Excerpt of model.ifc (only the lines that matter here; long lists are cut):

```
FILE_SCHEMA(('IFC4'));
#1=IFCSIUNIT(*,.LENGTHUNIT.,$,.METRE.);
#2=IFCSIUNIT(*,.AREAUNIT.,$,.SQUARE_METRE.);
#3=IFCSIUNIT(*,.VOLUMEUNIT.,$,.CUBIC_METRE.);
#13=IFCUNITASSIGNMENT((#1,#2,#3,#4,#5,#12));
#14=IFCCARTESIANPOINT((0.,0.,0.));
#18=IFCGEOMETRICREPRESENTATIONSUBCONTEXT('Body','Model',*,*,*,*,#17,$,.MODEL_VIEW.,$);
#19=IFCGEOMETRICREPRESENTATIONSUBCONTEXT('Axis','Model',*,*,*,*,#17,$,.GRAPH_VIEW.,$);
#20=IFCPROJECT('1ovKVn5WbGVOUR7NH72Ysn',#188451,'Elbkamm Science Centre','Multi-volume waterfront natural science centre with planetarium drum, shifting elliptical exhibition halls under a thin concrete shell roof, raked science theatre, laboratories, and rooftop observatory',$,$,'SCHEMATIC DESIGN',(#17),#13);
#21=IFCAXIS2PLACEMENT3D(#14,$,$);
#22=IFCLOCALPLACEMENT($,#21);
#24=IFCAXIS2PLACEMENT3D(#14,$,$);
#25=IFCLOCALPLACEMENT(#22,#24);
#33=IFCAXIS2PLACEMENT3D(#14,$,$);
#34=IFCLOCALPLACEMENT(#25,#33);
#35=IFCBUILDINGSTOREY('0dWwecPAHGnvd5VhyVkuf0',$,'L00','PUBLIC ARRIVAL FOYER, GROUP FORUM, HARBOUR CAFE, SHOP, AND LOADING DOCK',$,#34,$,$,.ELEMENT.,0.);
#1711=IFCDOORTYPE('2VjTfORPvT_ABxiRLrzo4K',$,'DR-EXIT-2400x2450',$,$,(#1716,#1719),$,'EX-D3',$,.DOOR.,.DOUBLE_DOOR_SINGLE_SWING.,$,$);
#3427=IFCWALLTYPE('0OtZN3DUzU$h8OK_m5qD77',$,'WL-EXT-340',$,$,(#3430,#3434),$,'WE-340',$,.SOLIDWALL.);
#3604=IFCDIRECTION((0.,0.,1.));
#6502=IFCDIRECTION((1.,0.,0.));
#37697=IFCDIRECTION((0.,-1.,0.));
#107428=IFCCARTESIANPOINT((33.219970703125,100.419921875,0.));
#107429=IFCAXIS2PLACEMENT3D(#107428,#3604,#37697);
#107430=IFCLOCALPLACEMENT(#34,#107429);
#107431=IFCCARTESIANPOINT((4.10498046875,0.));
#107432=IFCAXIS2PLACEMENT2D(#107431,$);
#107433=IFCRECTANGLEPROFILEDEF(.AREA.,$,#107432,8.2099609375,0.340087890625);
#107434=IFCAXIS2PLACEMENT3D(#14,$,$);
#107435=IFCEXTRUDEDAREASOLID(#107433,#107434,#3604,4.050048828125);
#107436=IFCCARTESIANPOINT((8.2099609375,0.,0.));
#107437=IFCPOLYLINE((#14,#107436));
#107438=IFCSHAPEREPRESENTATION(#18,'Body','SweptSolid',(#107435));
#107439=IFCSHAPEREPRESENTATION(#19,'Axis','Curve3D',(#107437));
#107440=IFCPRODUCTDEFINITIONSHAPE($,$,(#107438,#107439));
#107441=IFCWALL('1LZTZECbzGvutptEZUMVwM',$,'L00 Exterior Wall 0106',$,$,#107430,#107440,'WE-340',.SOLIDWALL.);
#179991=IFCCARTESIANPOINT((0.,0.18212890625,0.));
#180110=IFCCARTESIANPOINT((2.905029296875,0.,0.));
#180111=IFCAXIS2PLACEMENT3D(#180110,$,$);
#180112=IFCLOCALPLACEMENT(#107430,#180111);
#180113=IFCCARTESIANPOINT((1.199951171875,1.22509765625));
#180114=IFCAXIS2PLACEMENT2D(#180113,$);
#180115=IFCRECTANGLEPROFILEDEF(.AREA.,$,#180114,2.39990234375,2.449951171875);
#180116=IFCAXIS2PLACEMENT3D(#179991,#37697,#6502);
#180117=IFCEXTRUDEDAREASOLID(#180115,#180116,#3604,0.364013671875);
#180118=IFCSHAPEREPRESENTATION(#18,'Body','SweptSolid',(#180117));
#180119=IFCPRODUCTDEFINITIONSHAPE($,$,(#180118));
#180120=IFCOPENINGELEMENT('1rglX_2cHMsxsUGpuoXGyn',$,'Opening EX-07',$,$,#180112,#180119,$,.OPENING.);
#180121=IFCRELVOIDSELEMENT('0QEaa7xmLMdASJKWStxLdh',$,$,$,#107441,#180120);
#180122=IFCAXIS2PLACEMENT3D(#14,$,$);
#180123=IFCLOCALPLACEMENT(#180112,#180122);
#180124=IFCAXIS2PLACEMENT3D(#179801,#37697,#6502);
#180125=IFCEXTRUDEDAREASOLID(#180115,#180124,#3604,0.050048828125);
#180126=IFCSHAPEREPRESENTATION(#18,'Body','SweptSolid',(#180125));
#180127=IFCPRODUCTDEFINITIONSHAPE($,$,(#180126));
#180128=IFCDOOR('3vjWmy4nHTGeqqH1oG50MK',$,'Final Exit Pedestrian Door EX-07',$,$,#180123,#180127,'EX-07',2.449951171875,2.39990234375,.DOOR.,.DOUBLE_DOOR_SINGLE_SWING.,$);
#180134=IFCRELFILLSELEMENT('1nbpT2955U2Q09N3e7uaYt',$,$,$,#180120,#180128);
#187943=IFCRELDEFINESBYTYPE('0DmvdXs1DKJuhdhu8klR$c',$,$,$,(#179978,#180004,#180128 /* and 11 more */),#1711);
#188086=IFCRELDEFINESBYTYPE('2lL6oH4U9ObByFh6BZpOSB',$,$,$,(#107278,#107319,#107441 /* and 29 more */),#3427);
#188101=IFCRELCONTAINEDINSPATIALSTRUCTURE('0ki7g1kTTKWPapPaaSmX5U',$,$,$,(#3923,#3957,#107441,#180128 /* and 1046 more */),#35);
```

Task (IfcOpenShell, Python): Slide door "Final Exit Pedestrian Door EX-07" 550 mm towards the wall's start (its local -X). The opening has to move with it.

```python
import ifcopenshell
import ifcopenshell.api.geometry
import ifcopenshell.util.placement
import ifcopenshell.util.unit

model = ifcopenshell.open("model.ifc")
unit_scale = ifcopenshell.util.unit.calculate_unit_scale(model)

door = model.by_guid("3vjWmy4nHTGeqqH1oG50MK")
opening = door.FillsVoids[0].RelatingOpeningElement
wall = opening.VoidsElements[0].RelatingBuildingElement

wall_matrix = ifcopenshell.util.placement.get_local_placement(wall.ObjectPlacement)
shift = wall_matrix[:3, 0] * -0.55 / unit_scale
before = ifcopenshell.util.placement.get_local_placement(door.ObjectPlacement)[:3, 3].copy()

# The door is placed relative to its opening, so it follows when the opening moves.
matrix = ifcopenshell.util.placement.get_local_placement(opening.ObjectPlacement)
matrix[:3, 3] += shift
ifcopenshell.api.geometry.edit_object_placement(
    model, product=opening, matrix=matrix, is_si=False, should_transform_children=True
)

after = ifcopenshell.util.placement.get_local_placement(door.ObjectPlacement)[:3, 3]
print("door moved by", (after - before).round(3) + 0.0)

model.write("model_updated.ifc")
```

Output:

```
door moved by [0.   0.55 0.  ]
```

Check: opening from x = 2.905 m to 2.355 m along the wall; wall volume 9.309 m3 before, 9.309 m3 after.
